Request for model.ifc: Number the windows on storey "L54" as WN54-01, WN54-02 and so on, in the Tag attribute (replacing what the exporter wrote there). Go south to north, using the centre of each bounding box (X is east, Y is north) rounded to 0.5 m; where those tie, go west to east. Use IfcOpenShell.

First a look at what the model holds.

```python
import ifcopenshell
import ifcopenshell.util.element
import ifcopenshell.util.placement

model = ifcopenshell.open("model.ifc")
print(model.schema)
storey = next(s for s in model.by_type("IfcBuildingStorey") if s.Name == "L54")
windows = [e for e in ifcopenshell.util.element.get_decomposition(storey) if e.is_a("IfcWindow")]
for e in sorted(windows, key=lambda e: e.id()):
    origin = ifcopenshell.util.placement.get_local_placement(e.ObjectPlacement)[:3, 3]
    print(e.id(), e.Tag, e.Name, origin.round(2) + 0.0, sep=" | ")
```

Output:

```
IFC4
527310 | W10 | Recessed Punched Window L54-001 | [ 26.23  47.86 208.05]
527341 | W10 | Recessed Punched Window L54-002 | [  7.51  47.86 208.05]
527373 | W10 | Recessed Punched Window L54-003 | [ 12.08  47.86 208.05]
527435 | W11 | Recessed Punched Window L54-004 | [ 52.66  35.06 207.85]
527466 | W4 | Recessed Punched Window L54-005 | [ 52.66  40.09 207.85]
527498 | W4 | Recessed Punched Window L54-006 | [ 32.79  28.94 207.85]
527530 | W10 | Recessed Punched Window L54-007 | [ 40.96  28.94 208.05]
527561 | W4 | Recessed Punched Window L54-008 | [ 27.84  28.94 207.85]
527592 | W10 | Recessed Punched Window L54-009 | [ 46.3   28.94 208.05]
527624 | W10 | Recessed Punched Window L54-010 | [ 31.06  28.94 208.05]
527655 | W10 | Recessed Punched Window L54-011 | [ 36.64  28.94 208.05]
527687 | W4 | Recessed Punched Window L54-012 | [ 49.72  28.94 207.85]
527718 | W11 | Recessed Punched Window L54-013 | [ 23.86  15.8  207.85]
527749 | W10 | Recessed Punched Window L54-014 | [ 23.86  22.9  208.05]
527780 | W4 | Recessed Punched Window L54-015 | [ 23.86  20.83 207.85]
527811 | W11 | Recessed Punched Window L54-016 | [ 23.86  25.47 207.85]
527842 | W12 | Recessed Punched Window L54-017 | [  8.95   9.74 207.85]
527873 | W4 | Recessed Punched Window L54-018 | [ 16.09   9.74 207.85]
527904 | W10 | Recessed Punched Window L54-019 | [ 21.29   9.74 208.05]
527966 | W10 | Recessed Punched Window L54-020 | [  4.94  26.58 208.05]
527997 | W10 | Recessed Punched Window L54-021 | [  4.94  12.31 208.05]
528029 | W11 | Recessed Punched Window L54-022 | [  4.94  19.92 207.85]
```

```python
import ifcopenshell
import ifcopenshell.geom
import ifcopenshell.util.element
import ifcopenshell.util.shape

model = ifcopenshell.open("model.ifc")
settings = ifcopenshell.geom.settings()
settings.set("use-world-coords", True)


def centre(element):
    shape = ifcopenshell.geom.create_shape(settings, element)
    return ifcopenshell.util.shape.get_bbox_centroid(shape.geometry)


storey = next(s for s in model.by_type("IfcBuildingStorey") if s.Name == "L54")
windows = [e for e in ifcopenshell.util.element.get_decomposition(storey) if e.is_a("IfcWindow")]

# Insertion points can sit at a corner or the storey origin, so sort by the geometry (in metres).
centres = {e: centre(e) for e in windows}
windows.sort(key=lambda e: (round(centres[e][1] / 0.5), centres[e][0]))

for i, e in enumerate(windows, start=1):
    number = f"WN54-{i:02d}"
    e.Tag = number
    print(e.id(), number)

model.write("model_rev.ifc")
```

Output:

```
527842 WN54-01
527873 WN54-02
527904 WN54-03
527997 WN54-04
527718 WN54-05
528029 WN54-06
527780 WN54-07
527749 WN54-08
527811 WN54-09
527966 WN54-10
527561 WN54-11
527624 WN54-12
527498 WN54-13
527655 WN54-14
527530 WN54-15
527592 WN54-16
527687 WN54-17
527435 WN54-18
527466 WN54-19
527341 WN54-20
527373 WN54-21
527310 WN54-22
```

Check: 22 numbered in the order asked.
